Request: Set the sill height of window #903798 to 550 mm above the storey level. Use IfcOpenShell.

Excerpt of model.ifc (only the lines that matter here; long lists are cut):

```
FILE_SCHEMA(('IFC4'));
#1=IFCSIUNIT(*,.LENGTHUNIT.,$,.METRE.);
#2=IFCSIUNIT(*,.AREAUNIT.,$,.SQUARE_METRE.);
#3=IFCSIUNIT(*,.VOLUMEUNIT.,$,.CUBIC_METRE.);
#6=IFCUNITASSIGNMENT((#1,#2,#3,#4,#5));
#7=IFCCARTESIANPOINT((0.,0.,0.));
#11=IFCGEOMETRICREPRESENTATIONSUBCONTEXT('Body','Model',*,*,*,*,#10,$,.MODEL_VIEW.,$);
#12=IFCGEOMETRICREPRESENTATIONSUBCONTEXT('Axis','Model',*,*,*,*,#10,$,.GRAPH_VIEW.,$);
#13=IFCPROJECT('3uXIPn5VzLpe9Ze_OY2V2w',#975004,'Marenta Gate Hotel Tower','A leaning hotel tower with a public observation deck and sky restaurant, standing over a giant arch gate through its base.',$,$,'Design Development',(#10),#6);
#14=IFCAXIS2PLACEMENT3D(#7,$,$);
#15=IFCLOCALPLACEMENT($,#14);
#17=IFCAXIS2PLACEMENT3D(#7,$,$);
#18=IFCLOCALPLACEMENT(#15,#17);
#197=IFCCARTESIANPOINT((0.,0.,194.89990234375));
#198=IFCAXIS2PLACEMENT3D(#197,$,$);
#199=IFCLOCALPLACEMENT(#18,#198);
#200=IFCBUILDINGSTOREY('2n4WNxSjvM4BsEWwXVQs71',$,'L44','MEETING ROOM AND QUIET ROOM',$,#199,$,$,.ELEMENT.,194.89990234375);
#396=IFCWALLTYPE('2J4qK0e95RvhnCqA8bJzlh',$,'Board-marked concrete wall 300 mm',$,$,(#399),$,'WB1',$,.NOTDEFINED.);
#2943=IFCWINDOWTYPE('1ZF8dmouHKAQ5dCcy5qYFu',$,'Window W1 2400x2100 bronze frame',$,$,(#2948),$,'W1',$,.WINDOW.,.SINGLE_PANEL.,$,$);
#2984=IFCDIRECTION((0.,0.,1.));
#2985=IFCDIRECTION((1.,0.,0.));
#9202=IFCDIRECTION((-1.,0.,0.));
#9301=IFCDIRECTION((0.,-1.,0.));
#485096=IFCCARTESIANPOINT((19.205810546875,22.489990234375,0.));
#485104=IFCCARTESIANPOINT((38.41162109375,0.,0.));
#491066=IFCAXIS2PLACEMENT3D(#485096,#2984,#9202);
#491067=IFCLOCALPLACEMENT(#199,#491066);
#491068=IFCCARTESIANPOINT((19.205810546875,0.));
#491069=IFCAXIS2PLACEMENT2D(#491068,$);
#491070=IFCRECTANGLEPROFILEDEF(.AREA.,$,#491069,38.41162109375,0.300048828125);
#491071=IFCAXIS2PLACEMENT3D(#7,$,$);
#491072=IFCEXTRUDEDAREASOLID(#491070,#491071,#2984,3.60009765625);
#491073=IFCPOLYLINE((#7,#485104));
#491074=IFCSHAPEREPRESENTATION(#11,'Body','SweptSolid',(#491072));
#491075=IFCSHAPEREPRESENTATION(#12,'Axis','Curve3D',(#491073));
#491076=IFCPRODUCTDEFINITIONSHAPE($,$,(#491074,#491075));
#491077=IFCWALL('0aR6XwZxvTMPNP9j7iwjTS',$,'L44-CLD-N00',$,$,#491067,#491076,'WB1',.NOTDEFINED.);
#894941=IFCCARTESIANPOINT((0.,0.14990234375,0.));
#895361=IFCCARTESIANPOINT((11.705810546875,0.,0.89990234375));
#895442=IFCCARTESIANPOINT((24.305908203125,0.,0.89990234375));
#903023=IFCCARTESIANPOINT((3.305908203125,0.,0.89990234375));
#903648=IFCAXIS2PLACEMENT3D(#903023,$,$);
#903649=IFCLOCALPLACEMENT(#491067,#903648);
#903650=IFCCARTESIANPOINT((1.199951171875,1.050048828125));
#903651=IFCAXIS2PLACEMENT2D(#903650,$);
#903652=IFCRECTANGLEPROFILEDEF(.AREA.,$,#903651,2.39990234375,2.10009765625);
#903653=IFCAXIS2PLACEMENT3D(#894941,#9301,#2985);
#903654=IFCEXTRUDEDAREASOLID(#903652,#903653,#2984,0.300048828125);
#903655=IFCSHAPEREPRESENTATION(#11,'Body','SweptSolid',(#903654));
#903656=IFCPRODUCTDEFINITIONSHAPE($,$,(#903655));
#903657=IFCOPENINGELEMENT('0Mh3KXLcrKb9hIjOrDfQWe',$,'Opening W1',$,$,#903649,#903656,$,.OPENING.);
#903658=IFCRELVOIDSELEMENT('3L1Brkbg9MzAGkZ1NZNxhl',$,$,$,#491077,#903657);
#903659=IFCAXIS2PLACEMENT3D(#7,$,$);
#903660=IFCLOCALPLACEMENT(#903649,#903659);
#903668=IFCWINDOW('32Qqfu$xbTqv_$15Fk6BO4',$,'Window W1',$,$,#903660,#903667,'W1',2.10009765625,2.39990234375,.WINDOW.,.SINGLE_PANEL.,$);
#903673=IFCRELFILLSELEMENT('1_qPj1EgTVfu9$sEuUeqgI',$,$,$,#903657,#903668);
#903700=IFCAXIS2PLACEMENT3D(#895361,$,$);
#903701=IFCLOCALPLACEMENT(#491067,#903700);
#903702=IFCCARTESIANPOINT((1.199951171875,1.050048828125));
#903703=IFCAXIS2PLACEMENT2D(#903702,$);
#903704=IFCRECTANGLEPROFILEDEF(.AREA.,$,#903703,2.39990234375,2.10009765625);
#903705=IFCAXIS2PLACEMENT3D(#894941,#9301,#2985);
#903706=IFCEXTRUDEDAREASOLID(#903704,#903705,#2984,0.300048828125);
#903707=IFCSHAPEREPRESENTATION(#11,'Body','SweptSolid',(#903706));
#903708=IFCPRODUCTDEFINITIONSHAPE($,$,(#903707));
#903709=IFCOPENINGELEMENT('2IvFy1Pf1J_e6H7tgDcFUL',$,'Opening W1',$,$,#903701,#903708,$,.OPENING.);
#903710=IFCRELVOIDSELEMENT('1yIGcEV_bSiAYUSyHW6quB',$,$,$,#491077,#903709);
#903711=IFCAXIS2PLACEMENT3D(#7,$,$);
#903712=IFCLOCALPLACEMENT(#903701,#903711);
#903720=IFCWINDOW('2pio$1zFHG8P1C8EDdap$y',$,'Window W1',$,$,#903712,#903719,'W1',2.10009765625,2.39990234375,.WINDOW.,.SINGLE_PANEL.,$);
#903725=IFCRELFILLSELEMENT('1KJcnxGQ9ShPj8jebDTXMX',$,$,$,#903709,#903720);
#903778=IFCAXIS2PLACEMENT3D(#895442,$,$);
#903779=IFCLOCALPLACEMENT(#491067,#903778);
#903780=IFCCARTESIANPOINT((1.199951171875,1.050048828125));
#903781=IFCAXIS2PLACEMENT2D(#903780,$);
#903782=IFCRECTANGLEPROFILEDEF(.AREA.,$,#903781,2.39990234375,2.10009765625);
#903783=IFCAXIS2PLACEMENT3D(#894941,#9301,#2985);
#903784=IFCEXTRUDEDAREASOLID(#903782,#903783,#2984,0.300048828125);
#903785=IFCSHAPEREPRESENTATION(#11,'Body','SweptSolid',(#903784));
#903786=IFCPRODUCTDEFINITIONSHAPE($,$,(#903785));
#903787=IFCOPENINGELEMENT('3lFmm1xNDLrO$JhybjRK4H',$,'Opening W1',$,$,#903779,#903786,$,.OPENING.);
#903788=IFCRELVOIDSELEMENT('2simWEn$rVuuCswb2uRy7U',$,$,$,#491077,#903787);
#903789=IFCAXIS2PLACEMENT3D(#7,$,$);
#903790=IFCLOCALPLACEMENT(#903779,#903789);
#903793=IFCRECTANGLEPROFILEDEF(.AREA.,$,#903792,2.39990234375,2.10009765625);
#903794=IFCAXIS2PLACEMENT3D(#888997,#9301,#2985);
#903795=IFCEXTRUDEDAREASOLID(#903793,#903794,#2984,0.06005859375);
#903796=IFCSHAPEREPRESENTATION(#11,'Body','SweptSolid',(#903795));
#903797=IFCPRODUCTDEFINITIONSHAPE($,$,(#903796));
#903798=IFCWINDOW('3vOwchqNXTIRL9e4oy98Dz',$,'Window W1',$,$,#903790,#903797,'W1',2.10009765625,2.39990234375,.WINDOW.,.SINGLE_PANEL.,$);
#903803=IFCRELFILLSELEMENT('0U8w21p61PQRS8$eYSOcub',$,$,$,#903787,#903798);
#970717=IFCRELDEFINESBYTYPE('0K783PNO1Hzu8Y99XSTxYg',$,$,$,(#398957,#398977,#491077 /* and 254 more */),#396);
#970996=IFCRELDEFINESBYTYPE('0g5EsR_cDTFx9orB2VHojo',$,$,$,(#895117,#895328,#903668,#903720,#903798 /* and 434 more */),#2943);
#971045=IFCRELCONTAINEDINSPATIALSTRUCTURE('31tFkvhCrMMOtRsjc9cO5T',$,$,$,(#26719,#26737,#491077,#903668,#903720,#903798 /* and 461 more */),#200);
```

```python
import numpy as np
import ifcopenshell
import ifcopenshell.api.geometry
import ifcopenshell.geom
import ifcopenshell.util.element
import ifcopenshell.util.placement
import ifcopenshell.util.shape
import ifcopenshell.util.unit

model = ifcopenshell.open("model.ifc")
unit_scale = ifcopenshell.util.unit.calculate_unit_scale(model)

window = model.by_guid("3vOwchqNXTIRL9e4oy98Dz")
opening = window.FillsVoids[0].RelatingOpeningElement
storey = ifcopenshell.util.element.get_container(window, ifc_class="IfcBuildingStorey")
level = ifcopenshell.util.placement.get_local_placement(storey.ObjectPlacement)[2, 3]

# The opening's origin need not be at the sill, so measure its lowest point.
shape = ifcopenshell.geom.create_shape(ifcopenshell.geom.settings(), opening)
bottom = ifcopenshell.util.shape.get_shape_bottom_elevation(shape, shape.geometry) / unit_scale
dz = level + 0.55 / unit_scale - bottom

shift = np.array([0.0, 0.0, dz])
# The window is placed relative to its opening, so it follows when the opening moves.
matrix = ifcopenshell.util.placement.get_local_placement(opening.ObjectPlacement)
matrix[:3, 3] += shift
ifcopenshell.api.geometry.edit_object_placement(
    model, product=opening, matrix=matrix, is_si=False, should_transform_children=True
)

print(f"moved by {dz * unit_scale:+.3f} m")

model.write("model_v2.ifc")
```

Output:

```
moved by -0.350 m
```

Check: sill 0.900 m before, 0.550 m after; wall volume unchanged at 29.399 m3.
